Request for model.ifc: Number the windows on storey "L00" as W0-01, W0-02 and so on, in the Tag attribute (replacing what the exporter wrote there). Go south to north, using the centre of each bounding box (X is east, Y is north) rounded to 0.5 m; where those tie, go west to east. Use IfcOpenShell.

First a look at what the model holds.

```python
import ifcopenshell
import ifcopenshell.util.element
import ifcopenshell.util.placement

model = ifcopenshell.open("model.ifc")
print(model.schema)
storey = next(s for s in model.by_type("IfcBuildingStorey") if s.Name == "L00")
windows = [e for e in ifcopenshell.util.element.get_decomposition(storey) if e.is_a("IfcWindow")]
for e in sorted(windows, key=lambda e: e.id()):
    origin = ifcopenshell.util.placement.get_local_placement(e.ObjectPlacement)[:3, 3]
    print(e.id(), e.Tag, e.Name, origin.round(2) + 0.0, sep=" | ")
```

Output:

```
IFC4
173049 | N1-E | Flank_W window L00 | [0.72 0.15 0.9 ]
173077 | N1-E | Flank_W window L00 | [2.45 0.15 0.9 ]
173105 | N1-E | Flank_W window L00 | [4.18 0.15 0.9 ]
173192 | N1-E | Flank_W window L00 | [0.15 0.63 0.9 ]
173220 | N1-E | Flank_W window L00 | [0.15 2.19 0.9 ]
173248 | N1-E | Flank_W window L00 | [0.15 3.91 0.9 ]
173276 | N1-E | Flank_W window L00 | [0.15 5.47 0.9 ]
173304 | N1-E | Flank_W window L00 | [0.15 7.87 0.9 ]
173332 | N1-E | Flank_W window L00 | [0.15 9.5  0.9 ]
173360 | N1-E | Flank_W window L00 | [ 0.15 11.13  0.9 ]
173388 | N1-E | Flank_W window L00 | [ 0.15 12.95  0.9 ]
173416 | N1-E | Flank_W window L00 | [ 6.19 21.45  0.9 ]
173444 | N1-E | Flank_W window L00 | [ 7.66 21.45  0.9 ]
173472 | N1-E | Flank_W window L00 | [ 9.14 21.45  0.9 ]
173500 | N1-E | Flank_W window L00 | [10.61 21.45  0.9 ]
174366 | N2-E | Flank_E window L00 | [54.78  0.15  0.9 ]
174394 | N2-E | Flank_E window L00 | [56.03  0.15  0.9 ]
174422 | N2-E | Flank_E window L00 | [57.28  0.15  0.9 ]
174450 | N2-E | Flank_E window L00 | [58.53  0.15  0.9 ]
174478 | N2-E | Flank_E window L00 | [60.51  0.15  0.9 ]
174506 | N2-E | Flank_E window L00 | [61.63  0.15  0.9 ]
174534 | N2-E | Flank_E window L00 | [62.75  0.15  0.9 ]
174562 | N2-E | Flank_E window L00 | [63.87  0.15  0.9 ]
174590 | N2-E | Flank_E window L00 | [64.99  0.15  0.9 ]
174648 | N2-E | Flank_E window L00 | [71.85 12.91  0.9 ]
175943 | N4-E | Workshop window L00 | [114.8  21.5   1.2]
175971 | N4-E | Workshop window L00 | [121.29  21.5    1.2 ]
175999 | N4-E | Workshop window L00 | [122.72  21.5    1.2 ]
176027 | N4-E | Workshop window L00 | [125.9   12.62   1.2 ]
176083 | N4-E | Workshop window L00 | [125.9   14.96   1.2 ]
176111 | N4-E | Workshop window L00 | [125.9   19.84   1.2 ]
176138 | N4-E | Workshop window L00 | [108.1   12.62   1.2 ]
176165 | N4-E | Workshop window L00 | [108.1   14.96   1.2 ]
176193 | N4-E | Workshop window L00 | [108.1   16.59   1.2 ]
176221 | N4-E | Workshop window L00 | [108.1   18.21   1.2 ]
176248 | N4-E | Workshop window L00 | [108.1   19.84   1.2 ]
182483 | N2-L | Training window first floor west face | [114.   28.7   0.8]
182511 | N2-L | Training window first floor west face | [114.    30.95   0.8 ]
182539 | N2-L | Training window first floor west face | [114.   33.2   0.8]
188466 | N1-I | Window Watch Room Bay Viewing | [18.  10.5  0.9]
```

```python
import ifcopenshell
import ifcopenshell.geom
import ifcopenshell.util.element
import ifcopenshell.util.shape

model = ifcopenshell.open("model.ifc")
settings = ifcopenshell.geom.settings()
settings.set("use-world-coords", True)


def centre(element):
    shape = ifcopenshell.geom.create_shape(settings, element)
    return ifcopenshell.util.shape.get_bbox_centroid(shape.geometry)


storey = next(s for s in model.by_type("IfcBuildingStorey") if s.Name == "L00")
windows = [e for e in ifcopenshell.util.element.get_decomposition(storey) if e.is_a("IfcWindow")]

# Insertion points can sit at a corner or the storey origin, so sort by the geometry (in metres).
centres = {e: centre(e) for e in windows}
windows.sort(key=lambda e: (round(centres[e][1] / 0.5), centres[e][0]))

for i, e in enumerate(windows, start=1):
    number = f"W0-{i:02d}"
    e.Tag = number
    print(e.id(), number)

model.write("model_v2.ifc")
```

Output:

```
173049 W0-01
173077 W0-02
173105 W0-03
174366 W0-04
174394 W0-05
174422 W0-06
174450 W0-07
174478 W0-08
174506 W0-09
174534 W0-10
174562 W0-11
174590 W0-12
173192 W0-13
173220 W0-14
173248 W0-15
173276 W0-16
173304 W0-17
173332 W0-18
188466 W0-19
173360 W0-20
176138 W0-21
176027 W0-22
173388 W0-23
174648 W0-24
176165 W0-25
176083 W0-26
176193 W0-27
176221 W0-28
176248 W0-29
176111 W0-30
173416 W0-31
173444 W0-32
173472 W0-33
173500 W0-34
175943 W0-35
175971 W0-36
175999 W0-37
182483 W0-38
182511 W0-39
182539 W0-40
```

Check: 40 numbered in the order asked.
